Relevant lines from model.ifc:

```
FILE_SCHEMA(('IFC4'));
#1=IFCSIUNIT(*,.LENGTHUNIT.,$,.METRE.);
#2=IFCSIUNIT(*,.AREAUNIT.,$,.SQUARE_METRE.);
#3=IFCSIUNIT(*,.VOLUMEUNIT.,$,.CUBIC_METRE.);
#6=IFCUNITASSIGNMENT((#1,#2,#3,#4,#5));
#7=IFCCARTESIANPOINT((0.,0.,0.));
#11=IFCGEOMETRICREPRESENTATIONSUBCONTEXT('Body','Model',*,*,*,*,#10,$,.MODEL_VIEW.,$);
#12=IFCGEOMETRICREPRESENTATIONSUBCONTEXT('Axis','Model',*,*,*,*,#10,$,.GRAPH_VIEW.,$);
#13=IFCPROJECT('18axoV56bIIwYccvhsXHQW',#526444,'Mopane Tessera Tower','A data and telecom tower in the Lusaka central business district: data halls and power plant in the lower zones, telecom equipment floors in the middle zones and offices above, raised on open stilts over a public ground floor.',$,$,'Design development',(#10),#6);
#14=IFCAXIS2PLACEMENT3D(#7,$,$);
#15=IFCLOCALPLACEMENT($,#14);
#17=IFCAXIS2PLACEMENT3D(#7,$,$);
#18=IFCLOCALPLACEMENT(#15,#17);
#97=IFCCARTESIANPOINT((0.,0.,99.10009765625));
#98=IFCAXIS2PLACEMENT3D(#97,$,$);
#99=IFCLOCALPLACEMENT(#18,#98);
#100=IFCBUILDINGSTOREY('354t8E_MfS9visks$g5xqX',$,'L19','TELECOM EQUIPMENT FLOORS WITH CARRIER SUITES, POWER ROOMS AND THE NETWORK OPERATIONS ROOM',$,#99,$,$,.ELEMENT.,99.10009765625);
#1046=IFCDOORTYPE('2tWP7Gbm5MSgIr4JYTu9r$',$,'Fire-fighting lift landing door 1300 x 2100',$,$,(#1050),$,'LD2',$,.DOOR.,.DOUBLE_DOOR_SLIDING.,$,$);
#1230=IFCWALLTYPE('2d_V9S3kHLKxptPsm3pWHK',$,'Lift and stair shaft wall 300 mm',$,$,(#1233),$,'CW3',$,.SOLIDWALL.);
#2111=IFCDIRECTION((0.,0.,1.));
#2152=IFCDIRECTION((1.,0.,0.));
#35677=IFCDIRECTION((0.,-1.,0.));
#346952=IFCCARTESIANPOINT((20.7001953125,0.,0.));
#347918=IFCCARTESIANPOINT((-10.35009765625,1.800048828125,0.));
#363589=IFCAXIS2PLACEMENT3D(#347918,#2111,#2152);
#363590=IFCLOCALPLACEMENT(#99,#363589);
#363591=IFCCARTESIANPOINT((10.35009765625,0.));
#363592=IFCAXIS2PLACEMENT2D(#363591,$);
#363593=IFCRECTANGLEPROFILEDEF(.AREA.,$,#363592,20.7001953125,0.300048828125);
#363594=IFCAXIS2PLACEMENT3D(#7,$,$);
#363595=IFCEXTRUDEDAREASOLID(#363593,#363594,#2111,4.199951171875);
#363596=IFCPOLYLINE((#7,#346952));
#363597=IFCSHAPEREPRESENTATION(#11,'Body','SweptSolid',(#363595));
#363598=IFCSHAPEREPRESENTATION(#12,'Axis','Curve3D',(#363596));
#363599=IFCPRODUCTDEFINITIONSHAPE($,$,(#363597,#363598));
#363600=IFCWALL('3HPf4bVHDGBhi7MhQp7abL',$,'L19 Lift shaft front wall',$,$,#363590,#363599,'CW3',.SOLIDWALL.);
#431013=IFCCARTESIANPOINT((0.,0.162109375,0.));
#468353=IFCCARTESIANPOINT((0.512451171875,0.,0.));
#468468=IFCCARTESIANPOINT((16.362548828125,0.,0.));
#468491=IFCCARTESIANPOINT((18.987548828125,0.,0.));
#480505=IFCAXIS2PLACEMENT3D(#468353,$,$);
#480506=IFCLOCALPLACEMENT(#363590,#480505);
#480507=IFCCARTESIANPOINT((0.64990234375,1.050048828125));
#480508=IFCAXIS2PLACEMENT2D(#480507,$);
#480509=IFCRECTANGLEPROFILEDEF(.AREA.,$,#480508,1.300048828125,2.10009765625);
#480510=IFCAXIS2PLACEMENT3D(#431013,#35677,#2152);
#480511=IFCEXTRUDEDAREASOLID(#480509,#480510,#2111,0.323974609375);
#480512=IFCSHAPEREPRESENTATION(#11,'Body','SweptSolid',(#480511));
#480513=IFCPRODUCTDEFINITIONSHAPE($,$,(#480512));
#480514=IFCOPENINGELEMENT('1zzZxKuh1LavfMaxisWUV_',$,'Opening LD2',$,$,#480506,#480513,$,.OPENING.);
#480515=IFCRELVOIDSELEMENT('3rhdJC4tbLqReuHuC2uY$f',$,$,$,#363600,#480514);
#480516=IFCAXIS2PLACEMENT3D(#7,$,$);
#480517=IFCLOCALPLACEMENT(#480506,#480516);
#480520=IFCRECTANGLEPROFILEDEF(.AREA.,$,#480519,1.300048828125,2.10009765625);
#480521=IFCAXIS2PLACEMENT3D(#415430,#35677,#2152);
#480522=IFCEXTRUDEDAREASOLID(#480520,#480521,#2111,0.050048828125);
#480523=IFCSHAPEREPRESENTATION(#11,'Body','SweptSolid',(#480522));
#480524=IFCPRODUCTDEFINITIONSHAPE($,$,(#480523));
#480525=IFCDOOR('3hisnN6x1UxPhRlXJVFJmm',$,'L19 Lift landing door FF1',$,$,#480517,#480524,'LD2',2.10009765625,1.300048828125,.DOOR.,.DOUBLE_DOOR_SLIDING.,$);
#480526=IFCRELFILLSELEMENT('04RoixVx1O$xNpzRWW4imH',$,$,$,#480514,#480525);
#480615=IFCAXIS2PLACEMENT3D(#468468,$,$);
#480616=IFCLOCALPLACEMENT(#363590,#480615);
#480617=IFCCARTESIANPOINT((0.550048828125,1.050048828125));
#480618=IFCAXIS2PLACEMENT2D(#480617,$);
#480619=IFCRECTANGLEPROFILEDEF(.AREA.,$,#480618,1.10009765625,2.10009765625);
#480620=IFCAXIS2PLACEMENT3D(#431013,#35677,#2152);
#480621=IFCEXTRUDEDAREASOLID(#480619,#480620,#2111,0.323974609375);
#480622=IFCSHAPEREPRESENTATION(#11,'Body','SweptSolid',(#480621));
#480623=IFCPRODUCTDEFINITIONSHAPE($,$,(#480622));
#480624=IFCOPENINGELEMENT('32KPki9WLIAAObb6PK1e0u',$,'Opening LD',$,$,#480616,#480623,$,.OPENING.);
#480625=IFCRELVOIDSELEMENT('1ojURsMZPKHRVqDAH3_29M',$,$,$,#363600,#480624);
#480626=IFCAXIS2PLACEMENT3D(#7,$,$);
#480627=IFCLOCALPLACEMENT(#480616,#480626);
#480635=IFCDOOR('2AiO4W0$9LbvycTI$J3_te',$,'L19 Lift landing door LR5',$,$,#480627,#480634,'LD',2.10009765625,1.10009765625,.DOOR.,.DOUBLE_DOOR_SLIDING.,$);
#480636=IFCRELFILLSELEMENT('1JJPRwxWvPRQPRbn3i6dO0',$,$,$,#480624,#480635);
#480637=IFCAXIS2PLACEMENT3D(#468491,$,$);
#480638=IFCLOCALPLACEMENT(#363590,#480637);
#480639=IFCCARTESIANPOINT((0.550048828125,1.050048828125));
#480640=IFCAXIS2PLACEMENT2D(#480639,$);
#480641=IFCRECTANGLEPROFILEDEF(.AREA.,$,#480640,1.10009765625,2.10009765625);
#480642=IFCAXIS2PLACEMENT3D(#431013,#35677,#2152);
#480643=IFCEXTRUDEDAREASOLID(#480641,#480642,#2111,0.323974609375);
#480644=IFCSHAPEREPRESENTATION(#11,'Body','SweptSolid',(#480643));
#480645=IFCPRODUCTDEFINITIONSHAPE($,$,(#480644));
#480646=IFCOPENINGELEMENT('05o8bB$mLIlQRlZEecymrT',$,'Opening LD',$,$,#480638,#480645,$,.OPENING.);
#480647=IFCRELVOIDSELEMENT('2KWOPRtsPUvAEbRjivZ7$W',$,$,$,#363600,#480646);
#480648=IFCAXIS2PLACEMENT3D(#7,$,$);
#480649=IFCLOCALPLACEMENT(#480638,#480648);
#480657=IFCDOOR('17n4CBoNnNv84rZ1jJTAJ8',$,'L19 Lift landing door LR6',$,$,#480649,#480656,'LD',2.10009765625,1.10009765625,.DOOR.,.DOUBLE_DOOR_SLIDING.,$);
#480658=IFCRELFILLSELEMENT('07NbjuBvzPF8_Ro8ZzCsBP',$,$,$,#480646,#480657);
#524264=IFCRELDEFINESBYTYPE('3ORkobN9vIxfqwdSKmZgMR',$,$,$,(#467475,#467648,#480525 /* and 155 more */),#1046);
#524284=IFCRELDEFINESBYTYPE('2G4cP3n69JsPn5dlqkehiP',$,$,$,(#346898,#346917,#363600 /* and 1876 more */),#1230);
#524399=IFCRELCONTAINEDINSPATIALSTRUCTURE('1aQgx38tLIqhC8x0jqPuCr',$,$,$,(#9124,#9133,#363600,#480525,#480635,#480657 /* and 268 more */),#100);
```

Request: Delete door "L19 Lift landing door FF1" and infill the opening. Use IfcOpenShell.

```python
import ifcopenshell
import ifcopenshell.api.feature
import ifcopenshell.api.root
import ifcopenshell.geom
import ifcopenshell.util.shape

model = ifcopenshell.open("model.ifc")
settings = ifcopenshell.geom.settings()


def volume(element):
    """Net volume in cubic metres, openings subtracted."""
    shape = ifcopenshell.geom.create_shape(settings, element)
    return ifcopenshell.util.shape.get_volume(shape.geometry)


door = model.by_guid("3hisnN6x1UxPhRlXJVFJmm")
opening = door.FillsVoids[0].RelatingOpeningElement
wall = opening.VoidsElements[0].RelatingBuildingElement
before = volume(wall)

ifcopenshell.api.root.remove_product(model, product=door)
ifcopenshell.api.feature.remove_feature(model, feature=opening)

after = volume(wall)

print(f"wall volume {before:.3f} -> {after:.3f} m3")

model.write("model_v2.ifc")
```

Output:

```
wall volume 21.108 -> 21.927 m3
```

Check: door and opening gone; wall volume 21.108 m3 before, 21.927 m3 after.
